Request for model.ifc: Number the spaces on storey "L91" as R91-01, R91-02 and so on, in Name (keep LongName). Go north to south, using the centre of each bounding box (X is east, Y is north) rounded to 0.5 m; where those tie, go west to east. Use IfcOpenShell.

First a look at what the model holds.

```python
import ifcopenshell
import ifcopenshell.util.element
import ifcopenshell.util.placement

model = ifcopenshell.open("model.ifc")
print(model.schema)
storey = next(s for s in model.by_type("IfcBuildingStorey") if s.Name == "L91")
spaces = [e for e in ifcopenshell.util.element.get_decomposition(storey) if e.is_a("IfcSpace")]
for e in sorted(spaces, key=lambda e: e.id()):
    origin = ifcopenshell.util.placement.get_local_placement(e.ObjectPlacement)[:3, 3]
    print(e.id(), e.Name, e.LongName, origin.round(2) + 0.0, sep=" | ")
```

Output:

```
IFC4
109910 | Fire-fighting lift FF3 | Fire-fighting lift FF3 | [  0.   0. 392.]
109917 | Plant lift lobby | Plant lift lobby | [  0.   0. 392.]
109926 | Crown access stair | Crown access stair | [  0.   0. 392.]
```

```python
import ifcopenshell
import ifcopenshell.geom
import ifcopenshell.util.element
import ifcopenshell.util.shape

model = ifcopenshell.open("model.ifc")
settings = ifcopenshell.geom.settings()
settings.set("use-world-coords", True)


def centre(element):
    shape = ifcopenshell.geom.create_shape(settings, element)
    return ifcopenshell.util.shape.get_bbox_centroid(shape.geometry)


storey = next(s for s in model.by_type("IfcBuildingStorey") if s.Name == "L91")
spaces = [e for e in ifcopenshell.util.element.get_decomposition(storey) if e.is_a("IfcSpace")]

# Insertion points can sit at a corner or the storey origin, so sort by the geometry (in metres).
centres = {e: centre(e) for e in spaces}
spaces.sort(key=lambda e: (-round(centres[e][1] / 0.5), centres[e][0]))

for i, e in enumerate(spaces, start=1):
    number = f"R91-{i:02d}"
    e.Name = number
    print(e.id(), number)

model.write("model_v2.ifc")
```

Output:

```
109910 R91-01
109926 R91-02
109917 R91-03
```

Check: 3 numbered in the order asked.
